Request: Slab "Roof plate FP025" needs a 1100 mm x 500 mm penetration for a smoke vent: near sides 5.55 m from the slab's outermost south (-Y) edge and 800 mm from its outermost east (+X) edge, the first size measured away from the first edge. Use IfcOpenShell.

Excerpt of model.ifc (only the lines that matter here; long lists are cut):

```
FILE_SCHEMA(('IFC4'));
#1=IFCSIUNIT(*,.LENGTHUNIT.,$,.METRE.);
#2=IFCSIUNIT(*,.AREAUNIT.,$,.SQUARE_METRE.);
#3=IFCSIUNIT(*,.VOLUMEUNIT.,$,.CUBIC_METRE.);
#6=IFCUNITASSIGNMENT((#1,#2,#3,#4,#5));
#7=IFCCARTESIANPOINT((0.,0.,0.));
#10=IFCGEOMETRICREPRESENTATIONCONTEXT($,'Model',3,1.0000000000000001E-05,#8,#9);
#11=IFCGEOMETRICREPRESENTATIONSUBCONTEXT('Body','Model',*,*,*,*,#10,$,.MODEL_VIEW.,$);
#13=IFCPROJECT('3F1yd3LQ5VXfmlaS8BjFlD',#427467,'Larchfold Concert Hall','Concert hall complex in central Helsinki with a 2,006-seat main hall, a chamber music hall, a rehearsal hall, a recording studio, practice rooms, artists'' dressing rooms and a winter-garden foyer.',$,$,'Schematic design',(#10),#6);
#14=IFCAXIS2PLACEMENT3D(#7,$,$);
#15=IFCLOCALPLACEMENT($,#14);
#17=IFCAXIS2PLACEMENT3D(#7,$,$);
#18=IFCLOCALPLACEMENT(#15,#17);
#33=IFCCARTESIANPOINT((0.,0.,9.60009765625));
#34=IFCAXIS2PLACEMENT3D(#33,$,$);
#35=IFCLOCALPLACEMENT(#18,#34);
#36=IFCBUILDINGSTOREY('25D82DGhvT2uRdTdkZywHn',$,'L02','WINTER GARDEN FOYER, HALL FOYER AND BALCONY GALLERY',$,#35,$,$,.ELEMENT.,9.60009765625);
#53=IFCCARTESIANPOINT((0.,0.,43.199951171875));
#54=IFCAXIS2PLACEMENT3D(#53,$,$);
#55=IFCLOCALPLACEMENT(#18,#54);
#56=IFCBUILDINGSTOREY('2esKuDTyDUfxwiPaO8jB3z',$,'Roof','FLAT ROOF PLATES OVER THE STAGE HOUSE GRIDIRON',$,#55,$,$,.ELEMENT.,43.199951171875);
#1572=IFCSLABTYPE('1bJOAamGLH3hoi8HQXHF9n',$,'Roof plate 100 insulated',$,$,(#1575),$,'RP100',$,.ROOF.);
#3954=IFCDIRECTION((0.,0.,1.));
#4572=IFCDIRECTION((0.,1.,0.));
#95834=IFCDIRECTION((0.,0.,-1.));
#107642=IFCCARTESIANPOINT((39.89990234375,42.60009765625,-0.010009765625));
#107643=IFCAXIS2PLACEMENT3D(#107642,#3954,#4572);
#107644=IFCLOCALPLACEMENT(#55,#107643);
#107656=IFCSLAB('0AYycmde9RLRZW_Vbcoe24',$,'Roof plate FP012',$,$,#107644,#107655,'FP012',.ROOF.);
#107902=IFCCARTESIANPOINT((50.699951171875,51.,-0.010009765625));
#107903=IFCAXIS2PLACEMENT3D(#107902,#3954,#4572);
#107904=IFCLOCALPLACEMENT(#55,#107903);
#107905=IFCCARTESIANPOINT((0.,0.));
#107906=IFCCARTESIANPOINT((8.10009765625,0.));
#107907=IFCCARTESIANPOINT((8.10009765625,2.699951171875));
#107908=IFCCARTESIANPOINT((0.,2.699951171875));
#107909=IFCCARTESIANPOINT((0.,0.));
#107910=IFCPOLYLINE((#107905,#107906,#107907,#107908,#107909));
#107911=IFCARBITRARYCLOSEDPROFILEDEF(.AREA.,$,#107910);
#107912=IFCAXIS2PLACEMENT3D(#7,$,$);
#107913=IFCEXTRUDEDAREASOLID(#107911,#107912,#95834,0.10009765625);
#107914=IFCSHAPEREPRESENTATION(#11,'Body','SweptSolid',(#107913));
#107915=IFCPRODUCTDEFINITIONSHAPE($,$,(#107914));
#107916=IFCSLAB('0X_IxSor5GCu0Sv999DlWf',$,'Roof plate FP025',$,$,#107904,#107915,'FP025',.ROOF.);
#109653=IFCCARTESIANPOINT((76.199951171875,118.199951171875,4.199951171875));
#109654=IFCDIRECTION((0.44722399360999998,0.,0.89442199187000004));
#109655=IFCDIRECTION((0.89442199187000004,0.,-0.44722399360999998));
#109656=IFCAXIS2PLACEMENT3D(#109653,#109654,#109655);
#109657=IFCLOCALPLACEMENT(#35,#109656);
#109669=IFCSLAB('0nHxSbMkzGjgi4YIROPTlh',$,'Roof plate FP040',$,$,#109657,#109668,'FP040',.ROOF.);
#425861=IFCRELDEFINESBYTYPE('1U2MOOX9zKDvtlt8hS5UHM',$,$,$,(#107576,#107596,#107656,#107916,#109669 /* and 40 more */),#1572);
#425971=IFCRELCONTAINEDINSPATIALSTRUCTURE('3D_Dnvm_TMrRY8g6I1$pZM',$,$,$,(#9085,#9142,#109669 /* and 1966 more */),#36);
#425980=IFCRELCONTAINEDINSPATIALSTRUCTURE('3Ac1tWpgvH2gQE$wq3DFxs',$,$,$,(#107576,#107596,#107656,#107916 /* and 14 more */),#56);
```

```python
import numpy as np
import ifcopenshell
import ifcopenshell.api.feature
import ifcopenshell.api.geometry
import ifcopenshell.api.root
import ifcopenshell.geom
import ifcopenshell.util.placement
import ifcopenshell.util.representation
import ifcopenshell.util.shape
import ifcopenshell.util.unit

model = ifcopenshell.open("model.ifc")
unit_scale = ifcopenshell.util.unit.calculate_unit_scale(model)
settings = ifcopenshell.geom.settings()


def volume(element):
    """Net volume in cubic metres, openings subtracted."""
    shape = ifcopenshell.geom.create_shape(settings, element)
    return ifcopenshell.util.shape.get_volume(shape.geometry)


slab = model.by_guid("0X_IxSor5GCu0Sv999DlWf")
before = volume(slab)

# Extent in the slab's own axes, in metres. The edges named are its -X and -Y sides.
slab_shape = ifcopenshell.geom.create_shape(settings, slab)
vertices = ifcopenshell.util.shape.get_vertices(slab_shape.geometry)
x_min, y_min, bottom = vertices.min(axis=0)
top = vertices[:, 2].max()

opening = ifcopenshell.api.root.create_entity(model, ifc_class="IfcOpeningElement", name="Smoke vent opening", predefined_type="OPENING")
context = ifcopenshell.util.representation.get_context(model, "Model", "Body", "MODEL_VIEW")
width, depth = 1.1, 0.5
outline = [(0.0, 0.0), (width, 0.0), (width, depth), (0.0, depth), (0.0, 0.0)]
# Overshoot both faces by 50 mm so the cut is clean.
shape = ifcopenshell.api.geometry.add_slab_representation(
    model, context=context, depth=top - bottom + 0.1, polyline=outline
)
ifcopenshell.api.geometry.assign_representation(model, product=opening, representation=shape)

matrix = ifcopenshell.util.placement.get_local_placement(slab.ObjectPlacement)
matrix[:, 3] = matrix @ np.append(np.array([x_min + 5.55, y_min + 0.8, bottom - 0.05]) / unit_scale, 1.0)
ifcopenshell.api.geometry.edit_object_placement(model, product=opening, matrix=matrix, is_si=False)
ifcopenshell.api.feature.add_feature(model, feature=opening, element=slab)

after = volume(slab)

print(f"slab volume {before:.3f} -> {after:.3f} m3")

model.write("model_edited.ifc")
```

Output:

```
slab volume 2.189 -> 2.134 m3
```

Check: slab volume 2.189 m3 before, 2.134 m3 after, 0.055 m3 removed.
